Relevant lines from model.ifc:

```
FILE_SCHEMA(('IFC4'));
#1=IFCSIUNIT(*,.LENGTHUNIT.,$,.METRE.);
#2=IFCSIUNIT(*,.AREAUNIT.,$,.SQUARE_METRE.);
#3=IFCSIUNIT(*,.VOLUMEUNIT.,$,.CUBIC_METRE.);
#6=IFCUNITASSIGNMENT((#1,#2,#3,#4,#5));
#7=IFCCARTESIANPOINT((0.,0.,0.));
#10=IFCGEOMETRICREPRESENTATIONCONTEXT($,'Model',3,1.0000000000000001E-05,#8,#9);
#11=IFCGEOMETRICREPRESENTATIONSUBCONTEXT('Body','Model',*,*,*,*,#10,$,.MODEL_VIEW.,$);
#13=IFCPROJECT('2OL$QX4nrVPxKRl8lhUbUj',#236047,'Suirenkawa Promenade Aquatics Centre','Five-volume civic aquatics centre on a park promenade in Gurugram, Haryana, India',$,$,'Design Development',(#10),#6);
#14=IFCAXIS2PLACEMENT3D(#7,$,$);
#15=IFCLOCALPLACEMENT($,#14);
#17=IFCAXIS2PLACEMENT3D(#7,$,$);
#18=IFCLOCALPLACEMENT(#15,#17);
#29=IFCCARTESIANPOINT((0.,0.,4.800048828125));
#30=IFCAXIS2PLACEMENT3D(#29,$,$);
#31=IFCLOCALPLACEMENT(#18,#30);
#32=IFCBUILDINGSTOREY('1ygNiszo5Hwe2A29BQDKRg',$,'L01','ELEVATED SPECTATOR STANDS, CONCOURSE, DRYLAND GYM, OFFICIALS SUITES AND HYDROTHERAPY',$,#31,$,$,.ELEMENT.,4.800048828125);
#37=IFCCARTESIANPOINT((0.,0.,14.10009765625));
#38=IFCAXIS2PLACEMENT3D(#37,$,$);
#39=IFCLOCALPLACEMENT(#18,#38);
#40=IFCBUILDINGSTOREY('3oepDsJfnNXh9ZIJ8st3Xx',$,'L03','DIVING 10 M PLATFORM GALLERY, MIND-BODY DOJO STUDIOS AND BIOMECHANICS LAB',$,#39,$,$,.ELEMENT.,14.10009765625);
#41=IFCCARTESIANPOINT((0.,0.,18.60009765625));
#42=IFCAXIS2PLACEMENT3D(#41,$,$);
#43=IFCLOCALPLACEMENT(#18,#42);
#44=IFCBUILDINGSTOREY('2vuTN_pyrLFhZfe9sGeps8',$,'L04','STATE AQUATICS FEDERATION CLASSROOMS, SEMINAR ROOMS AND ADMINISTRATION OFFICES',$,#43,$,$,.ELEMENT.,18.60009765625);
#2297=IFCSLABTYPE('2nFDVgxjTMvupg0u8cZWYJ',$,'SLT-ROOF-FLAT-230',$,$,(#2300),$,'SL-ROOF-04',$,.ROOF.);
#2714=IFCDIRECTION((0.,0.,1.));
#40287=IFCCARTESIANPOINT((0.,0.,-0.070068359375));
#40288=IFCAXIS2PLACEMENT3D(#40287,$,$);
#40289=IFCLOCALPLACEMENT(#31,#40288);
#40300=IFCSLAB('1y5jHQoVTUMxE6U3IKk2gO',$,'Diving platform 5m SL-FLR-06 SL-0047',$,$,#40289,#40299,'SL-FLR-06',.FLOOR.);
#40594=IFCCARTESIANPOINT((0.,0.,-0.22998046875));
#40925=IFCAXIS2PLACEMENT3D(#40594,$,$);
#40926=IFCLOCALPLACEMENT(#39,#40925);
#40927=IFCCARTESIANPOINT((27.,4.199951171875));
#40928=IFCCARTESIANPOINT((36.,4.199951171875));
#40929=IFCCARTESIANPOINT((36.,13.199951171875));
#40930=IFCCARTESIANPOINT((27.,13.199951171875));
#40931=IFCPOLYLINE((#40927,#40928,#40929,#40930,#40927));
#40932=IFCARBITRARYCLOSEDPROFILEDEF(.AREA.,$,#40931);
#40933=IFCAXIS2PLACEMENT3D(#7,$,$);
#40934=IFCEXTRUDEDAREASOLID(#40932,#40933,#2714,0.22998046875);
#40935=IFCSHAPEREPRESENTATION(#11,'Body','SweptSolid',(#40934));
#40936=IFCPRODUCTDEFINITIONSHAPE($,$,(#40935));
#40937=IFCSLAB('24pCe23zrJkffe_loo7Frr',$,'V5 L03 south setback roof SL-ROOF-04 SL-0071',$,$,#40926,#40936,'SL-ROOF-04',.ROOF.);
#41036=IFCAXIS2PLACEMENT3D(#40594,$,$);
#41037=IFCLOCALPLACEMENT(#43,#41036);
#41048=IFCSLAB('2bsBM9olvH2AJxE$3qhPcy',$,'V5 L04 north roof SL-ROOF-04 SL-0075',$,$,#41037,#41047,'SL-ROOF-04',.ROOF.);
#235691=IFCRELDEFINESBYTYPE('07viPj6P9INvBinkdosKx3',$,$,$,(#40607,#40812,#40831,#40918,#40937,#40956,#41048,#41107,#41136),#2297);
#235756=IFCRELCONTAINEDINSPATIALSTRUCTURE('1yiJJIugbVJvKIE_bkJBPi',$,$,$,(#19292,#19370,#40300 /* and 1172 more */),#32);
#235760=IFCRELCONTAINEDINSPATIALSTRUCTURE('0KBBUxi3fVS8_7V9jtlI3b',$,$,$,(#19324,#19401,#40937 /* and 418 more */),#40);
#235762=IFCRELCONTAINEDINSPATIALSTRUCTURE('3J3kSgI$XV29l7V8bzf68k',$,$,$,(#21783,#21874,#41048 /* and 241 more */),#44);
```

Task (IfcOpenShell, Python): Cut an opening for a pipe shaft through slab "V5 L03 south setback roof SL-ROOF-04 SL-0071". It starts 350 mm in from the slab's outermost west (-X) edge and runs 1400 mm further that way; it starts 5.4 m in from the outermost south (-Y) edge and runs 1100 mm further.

```python
import numpy as np
import ifcopenshell
import ifcopenshell.api.feature
import ifcopenshell.api.geometry
import ifcopenshell.api.root
import ifcopenshell.geom
import ifcopenshell.util.placement
import ifcopenshell.util.representation
import ifcopenshell.util.shape
import ifcopenshell.util.unit

model = ifcopenshell.open("model.ifc")
unit_scale = ifcopenshell.util.unit.calculate_unit_scale(model)
settings = ifcopenshell.geom.settings()


def volume(element):
    """Net volume in cubic metres, openings subtracted."""
    shape = ifcopenshell.geom.create_shape(settings, element)
    return ifcopenshell.util.shape.get_volume(shape.geometry)


slab = model.by_guid("24pCe23zrJkffe_loo7Frr")
before = volume(slab)

# Extent in the slab's own axes, in metres. The edges named are its -X and -Y sides.
slab_shape = ifcopenshell.geom.create_shape(settings, slab)
vertices = ifcopenshell.util.shape.get_vertices(slab_shape.geometry)
x_min, y_min, bottom = vertices.min(axis=0)
top = vertices[:, 2].max()

opening = ifcopenshell.api.root.create_entity(model, ifc_class="IfcOpeningElement", name="Pipe shaft opening", predefined_type="OPENING")
context = ifcopenshell.util.representation.get_context(model, "Model", "Body", "MODEL_VIEW")
width, depth = 1.4, 1.1
outline = [(0.0, 0.0), (width, 0.0), (width, depth), (0.0, depth), (0.0, 0.0)]
# Overshoot both faces by 50 mm so the cut is clean.
shape = ifcopenshell.api.geometry.add_slab_representation(
    model, context=context, depth=top - bottom + 0.1, polyline=outline
)
ifcopenshell.api.geometry.assign_representation(model, product=opening, representation=shape)

matrix = ifcopenshell.util.placement.get_local_placement(slab.ObjectPlacement)
matrix[:, 3] = matrix @ np.append(np.array([x_min + 0.35, y_min + 5.4, bottom - 0.05]) / unit_scale, 1.0)
ifcopenshell.api.geometry.edit_object_placement(model, product=opening, matrix=matrix, is_si=False)
ifcopenshell.api.feature.add_feature(model, feature=opening, element=slab)

after = volume(slab)

print(f"slab volume {before:.3f} -> {after:.3f} m3")

model.write("model_rev.ifc")
```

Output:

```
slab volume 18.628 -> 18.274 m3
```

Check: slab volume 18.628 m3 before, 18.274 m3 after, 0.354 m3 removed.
